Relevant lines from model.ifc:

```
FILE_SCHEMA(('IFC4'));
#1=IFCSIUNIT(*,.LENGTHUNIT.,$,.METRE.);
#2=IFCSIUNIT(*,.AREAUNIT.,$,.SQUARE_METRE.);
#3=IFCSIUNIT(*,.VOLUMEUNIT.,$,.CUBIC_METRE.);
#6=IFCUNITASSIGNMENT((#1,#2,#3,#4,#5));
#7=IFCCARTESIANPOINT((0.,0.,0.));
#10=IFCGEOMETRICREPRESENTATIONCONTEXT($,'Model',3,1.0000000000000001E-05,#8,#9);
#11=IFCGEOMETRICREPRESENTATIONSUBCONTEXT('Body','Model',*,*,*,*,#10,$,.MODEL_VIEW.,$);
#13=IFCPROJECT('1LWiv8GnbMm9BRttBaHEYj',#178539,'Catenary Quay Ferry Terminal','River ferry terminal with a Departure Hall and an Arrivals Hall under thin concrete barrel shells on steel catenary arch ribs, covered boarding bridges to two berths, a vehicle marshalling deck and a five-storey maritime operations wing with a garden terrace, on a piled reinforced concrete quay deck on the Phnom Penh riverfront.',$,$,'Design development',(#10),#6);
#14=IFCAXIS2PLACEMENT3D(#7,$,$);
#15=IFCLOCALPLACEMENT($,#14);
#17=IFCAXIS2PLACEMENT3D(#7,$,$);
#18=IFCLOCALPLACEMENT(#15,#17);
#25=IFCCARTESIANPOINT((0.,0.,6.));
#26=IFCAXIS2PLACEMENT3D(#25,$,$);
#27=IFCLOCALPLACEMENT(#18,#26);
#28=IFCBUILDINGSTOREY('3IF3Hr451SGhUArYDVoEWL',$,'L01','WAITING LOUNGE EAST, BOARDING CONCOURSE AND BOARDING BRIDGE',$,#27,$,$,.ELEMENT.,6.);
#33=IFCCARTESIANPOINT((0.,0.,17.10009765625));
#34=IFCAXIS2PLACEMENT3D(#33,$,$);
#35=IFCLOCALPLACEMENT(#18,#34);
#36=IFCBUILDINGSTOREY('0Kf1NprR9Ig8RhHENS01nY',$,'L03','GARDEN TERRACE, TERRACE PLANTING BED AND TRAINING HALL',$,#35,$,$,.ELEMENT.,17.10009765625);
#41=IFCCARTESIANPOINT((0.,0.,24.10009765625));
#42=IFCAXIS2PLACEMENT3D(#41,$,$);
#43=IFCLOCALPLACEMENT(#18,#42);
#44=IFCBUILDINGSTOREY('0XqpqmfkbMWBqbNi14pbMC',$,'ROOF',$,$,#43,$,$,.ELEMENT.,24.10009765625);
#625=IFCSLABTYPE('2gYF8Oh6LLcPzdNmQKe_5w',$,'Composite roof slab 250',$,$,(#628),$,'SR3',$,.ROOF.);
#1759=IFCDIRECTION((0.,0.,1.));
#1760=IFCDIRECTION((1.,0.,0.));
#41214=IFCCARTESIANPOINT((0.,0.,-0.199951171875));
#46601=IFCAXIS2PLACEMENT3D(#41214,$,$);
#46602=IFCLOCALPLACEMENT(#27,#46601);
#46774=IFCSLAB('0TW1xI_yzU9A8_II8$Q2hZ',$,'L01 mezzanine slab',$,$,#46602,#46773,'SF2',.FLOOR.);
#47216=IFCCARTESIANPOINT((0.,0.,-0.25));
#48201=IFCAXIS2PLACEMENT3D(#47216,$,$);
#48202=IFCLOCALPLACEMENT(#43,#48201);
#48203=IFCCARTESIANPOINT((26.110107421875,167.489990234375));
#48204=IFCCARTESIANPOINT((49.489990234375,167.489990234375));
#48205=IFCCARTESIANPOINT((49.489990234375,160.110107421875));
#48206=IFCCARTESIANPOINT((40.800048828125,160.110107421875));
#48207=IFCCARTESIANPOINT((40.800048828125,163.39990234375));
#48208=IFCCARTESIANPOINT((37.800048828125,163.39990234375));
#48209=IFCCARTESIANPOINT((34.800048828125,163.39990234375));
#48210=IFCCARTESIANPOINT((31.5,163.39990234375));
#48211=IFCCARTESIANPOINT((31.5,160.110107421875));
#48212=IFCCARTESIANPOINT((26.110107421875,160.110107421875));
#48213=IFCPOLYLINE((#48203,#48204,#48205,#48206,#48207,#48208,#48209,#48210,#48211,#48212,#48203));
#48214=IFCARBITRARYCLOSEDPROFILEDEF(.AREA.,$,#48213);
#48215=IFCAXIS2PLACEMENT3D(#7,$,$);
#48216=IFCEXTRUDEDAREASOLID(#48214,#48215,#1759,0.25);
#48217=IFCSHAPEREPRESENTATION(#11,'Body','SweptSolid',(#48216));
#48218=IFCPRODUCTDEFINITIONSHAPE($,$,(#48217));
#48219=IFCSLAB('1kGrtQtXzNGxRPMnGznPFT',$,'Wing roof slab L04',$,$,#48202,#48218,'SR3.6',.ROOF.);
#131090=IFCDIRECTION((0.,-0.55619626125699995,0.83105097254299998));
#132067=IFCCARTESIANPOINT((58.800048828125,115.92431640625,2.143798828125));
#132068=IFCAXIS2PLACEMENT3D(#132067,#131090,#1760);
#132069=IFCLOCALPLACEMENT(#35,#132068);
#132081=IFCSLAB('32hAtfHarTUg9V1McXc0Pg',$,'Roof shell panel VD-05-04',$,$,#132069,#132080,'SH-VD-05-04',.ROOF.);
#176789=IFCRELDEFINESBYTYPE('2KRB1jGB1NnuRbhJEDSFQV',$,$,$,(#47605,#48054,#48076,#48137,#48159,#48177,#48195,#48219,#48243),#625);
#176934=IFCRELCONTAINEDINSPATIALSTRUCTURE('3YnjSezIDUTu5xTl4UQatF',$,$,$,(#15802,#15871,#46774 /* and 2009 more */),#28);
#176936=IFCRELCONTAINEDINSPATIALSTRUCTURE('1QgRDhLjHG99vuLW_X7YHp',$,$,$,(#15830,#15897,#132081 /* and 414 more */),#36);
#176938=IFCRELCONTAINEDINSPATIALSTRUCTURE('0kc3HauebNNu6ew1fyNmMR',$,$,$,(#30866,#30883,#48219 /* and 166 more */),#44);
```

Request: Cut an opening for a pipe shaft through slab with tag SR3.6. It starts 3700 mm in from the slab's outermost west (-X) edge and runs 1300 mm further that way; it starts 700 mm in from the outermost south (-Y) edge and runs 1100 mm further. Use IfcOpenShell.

```python
import numpy as np
import ifcopenshell
import ifcopenshell.api.feature
import ifcopenshell.api.geometry
import ifcopenshell.api.root
import ifcopenshell.geom
import ifcopenshell.util.placement
import ifcopenshell.util.representation
import ifcopenshell.util.shape
import ifcopenshell.util.unit

model = ifcopenshell.open("model.ifc")
unit_scale = ifcopenshell.util.unit.calculate_unit_scale(model)
settings = ifcopenshell.geom.settings()


def volume(element):
    """Net volume in cubic metres, openings subtracted."""
    shape = ifcopenshell.geom.create_shape(settings, element)
    return ifcopenshell.util.shape.get_volume(shape.geometry)


slab = model.by_id(48219)
before = volume(slab)

# Extent in the slab's own axes, in metres. The edges named are its -X and -Y sides.
slab_shape = ifcopenshell.geom.create_shape(settings, slab)
vertices = ifcopenshell.util.shape.get_vertices(slab_shape.geometry)
x_min, y_min, bottom = vertices.min(axis=0)
top = vertices[:, 2].max()

opening = ifcopenshell.api.root.create_entity(model, ifc_class="IfcOpeningElement", name="Pipe shaft opening", predefined_type="OPENING")
context = ifcopenshell.util.representation.get_context(model, "Model", "Body", "MODEL_VIEW")
width, depth = 1.3, 1.1
outline = [(0.0, 0.0), (width, 0.0), (width, depth), (0.0, depth), (0.0, 0.0)]
# Overshoot both faces by 50 mm so the cut is clean.
shape = ifcopenshell.api.geometry.add_slab_representation(
    model, context=context, depth=top - bottom + 0.1, polyline=outline
)
ifcopenshell.api.geometry.assign_representation(model, product=opening, representation=shape)

matrix = ifcopenshell.util.placement.get_local_placement(slab.ObjectPlacement)
matrix[:, 3] = matrix @ np.append(np.array([x_min + 3.7, y_min + 0.7, bottom - 0.05]) / unit_scale, 1.0)
ifcopenshell.api.geometry.edit_object_placement(model, product=opening, matrix=matrix, is_si=False)
ifcopenshell.api.feature.add_feature(model, feature=opening, element=slab)

after = volume(slab)

print(f"slab volume {before:.3f} -> {after:.3f} m3")

model.write("model-out.ifc")
```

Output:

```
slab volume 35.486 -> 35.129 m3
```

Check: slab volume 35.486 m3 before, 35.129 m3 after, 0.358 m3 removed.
